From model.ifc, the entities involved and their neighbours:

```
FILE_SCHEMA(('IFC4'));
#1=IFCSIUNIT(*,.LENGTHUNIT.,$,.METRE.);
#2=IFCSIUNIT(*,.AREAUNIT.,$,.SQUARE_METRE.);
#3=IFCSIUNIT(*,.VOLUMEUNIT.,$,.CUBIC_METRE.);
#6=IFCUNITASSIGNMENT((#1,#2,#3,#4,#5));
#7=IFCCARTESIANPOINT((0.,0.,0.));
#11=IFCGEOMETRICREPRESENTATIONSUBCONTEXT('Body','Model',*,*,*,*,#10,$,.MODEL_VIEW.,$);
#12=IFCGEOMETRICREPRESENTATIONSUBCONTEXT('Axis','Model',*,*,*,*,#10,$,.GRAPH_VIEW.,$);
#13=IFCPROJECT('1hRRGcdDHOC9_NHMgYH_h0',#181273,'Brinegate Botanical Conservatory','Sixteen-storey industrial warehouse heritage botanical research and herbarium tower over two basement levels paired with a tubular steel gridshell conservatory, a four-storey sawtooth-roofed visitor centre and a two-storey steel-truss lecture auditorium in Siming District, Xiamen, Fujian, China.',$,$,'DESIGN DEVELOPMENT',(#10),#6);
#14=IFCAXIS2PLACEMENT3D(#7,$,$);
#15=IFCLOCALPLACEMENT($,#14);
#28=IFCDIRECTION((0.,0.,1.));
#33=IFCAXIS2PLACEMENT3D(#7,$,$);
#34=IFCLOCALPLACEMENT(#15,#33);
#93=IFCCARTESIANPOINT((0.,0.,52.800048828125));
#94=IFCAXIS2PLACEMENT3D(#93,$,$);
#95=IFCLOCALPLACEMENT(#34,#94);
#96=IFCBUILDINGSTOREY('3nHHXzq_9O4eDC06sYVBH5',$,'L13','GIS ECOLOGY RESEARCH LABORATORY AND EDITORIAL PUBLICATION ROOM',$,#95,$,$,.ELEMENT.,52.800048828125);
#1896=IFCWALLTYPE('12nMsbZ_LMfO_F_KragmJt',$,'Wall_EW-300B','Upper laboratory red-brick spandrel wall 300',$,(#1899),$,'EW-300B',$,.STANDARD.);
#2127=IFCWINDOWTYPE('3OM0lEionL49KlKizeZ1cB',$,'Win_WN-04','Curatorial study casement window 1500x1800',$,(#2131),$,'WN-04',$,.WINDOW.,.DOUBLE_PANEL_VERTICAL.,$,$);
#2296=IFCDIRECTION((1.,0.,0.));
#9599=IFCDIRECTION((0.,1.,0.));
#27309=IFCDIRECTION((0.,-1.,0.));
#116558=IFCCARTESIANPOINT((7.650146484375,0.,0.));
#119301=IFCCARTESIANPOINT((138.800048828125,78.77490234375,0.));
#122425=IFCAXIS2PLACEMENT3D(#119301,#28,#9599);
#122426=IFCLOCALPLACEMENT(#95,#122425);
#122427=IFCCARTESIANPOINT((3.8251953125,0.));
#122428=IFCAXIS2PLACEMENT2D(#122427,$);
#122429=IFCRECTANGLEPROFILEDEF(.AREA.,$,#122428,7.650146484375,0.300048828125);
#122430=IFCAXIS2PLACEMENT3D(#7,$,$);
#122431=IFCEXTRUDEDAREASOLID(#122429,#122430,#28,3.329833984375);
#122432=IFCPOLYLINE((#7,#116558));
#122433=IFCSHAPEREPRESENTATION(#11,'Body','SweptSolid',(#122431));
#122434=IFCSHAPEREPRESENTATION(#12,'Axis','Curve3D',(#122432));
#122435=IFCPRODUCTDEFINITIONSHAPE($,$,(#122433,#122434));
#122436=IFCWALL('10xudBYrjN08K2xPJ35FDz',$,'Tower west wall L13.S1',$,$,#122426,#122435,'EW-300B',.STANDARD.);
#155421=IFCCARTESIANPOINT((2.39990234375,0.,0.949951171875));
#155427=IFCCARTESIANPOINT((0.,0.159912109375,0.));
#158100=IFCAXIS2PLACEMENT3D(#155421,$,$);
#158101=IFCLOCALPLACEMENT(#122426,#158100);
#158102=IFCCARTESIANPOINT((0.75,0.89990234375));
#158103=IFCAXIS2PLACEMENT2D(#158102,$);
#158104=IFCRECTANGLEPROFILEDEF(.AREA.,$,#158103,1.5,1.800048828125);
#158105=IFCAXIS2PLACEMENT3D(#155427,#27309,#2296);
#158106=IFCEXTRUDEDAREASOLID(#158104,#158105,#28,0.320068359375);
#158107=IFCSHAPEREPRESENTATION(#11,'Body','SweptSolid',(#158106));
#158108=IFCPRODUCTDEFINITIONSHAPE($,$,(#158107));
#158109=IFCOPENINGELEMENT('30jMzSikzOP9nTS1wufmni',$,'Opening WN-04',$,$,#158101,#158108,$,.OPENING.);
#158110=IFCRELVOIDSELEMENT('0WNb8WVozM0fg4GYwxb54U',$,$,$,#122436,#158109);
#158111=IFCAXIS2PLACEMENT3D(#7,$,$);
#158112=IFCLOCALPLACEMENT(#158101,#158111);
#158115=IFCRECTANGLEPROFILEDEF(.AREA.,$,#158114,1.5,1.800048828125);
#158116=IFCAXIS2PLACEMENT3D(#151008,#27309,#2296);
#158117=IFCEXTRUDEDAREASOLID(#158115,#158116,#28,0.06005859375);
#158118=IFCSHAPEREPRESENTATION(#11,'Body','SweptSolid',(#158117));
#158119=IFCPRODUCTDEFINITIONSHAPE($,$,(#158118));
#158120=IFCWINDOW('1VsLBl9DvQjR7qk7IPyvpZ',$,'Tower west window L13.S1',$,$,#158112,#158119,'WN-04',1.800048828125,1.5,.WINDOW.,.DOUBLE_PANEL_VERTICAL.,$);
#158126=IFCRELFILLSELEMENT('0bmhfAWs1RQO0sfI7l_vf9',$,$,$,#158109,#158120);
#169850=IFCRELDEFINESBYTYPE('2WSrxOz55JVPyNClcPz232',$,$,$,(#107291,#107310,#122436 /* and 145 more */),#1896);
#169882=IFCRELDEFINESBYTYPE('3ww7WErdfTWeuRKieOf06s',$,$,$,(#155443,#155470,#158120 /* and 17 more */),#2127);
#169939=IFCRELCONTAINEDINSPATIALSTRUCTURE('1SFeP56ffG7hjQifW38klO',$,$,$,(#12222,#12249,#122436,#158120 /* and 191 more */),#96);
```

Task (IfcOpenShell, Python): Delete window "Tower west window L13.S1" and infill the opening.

```python
import ifcopenshell
import ifcopenshell.api.feature
import ifcopenshell.api.root
import ifcopenshell.geom
import ifcopenshell.util.shape

model = ifcopenshell.open("model.ifc")
settings = ifcopenshell.geom.settings()


def volume(element):
    """Net volume in cubic metres, openings subtracted."""
    shape = ifcopenshell.geom.create_shape(settings, element)
    return ifcopenshell.util.shape.get_volume(shape.geometry)


window = model.by_id(158120)
opening = window.FillsVoids[0].RelatingOpeningElement
wall = opening.VoidsElements[0].RelatingBuildingElement
before = volume(wall)

ifcopenshell.api.root.remove_product(model, product=window)
ifcopenshell.api.feature.remove_feature(model, feature=opening)

after = volume(wall)

print(f"wall volume {before:.3f} -> {after:.3f} m3")

model.write("model_v2.ifc")
```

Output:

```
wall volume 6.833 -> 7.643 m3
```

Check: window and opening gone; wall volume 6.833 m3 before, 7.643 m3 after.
